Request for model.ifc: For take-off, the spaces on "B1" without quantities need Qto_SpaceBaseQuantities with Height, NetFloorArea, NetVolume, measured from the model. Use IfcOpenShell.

First a look at what the model holds.

```python
import ifcopenshell
import ifcopenshell.util.element
import ifcopenshell.util.unit

model = ifcopenshell.open("model.ifc")
print(model.schema)
for unit_type in ("LENGTHUNIT", "AREAUNIT", "VOLUMEUNIT"):
    print(unit_type, ifcopenshell.util.unit.calculate_unit_scale(model, unit_type))
storey = next(s for s in model.by_type("IfcBuildingStorey") if s.Name == "B1")
spaces = [e for e in ifcopenshell.util.element.get_decomposition(storey) if e.is_a("IfcSpace")]
for e in sorted(spaces, key=lambda e: e.id()):
    print(e.id(), e.is_a(), e.Name, list(ifcopenshell.util.element.get_psets(e, qtos_only=True)), sep=" | ")
```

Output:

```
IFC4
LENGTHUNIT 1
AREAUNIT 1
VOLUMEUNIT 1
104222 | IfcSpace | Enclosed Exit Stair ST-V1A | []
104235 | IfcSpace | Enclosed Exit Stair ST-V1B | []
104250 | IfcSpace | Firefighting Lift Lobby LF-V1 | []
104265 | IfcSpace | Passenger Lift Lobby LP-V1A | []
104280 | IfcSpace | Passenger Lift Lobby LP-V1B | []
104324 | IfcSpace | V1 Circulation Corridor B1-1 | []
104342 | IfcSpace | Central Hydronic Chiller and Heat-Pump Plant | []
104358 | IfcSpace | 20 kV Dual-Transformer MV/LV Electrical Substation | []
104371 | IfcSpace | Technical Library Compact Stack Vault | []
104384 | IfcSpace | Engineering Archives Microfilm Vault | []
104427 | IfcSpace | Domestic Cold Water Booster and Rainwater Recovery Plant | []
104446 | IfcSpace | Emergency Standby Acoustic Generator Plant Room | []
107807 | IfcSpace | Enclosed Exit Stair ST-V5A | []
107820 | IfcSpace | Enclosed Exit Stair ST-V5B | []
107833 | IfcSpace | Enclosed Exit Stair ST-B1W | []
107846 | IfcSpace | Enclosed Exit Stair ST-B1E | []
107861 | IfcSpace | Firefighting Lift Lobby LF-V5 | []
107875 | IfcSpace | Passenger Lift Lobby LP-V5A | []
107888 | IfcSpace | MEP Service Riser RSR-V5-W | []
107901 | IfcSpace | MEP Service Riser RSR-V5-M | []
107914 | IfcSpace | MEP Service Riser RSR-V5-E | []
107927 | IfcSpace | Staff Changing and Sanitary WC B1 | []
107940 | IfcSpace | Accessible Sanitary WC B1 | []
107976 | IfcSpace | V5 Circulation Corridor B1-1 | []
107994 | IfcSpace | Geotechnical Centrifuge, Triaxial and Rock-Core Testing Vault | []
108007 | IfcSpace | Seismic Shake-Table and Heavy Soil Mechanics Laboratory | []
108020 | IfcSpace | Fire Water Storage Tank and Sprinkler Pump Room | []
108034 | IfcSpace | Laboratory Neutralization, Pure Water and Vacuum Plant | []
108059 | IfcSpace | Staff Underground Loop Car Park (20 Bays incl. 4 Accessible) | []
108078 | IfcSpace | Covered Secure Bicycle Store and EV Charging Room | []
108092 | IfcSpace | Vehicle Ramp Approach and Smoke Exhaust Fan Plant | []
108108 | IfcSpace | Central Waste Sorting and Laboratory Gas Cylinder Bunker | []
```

```python
import ifcopenshell
import ifcopenshell.api.pset
import ifcopenshell.geom
import ifcopenshell.util.element
import ifcopenshell.util.shape
import ifcopenshell.util.unit

model = ifcopenshell.open("model.ifc")
unit_scale = ifcopenshell.util.unit.calculate_unit_scale(model)
area_scale = ifcopenshell.util.unit.calculate_unit_scale(model, "AREAUNIT")
volume_scale = ifcopenshell.util.unit.calculate_unit_scale(model, "VOLUMEUNIT")
settings = ifcopenshell.geom.settings()

storey = next(s for s in model.by_type("IfcBuildingStorey") if s.Name == "B1")
spaces = [e for e in ifcopenshell.util.element.get_decomposition(storey) if e.is_a("IfcSpace")]

for e in sorted(spaces, key=lambda e: e.id()):
    if ifcopenshell.util.element.get_psets(e, qtos_only=True, should_inherit=False):
        continue
    # Geometry comes back in metres, in the element's own axes.
    shape = ifcopenshell.geom.create_shape(settings, e)
    values = {
        "Height": ifcopenshell.util.shape.get_z(shape.geometry) / unit_scale,
        "NetFloorArea": ifcopenshell.util.shape.get_footprint_area(shape.geometry) / area_scale,
        "NetVolume": ifcopenshell.util.shape.get_volume(shape.geometry) / volume_scale,
    }
    qto = ifcopenshell.api.pset.add_qto(model, product=e, name="Qto_SpaceBaseQuantities")
    ifcopenshell.api.pset.edit_qto(model, qto=qto, properties=values)
    print(e.id(), {k: round(v, 3) for k, v in values.items()})

model.write("model_edited.ifc")
```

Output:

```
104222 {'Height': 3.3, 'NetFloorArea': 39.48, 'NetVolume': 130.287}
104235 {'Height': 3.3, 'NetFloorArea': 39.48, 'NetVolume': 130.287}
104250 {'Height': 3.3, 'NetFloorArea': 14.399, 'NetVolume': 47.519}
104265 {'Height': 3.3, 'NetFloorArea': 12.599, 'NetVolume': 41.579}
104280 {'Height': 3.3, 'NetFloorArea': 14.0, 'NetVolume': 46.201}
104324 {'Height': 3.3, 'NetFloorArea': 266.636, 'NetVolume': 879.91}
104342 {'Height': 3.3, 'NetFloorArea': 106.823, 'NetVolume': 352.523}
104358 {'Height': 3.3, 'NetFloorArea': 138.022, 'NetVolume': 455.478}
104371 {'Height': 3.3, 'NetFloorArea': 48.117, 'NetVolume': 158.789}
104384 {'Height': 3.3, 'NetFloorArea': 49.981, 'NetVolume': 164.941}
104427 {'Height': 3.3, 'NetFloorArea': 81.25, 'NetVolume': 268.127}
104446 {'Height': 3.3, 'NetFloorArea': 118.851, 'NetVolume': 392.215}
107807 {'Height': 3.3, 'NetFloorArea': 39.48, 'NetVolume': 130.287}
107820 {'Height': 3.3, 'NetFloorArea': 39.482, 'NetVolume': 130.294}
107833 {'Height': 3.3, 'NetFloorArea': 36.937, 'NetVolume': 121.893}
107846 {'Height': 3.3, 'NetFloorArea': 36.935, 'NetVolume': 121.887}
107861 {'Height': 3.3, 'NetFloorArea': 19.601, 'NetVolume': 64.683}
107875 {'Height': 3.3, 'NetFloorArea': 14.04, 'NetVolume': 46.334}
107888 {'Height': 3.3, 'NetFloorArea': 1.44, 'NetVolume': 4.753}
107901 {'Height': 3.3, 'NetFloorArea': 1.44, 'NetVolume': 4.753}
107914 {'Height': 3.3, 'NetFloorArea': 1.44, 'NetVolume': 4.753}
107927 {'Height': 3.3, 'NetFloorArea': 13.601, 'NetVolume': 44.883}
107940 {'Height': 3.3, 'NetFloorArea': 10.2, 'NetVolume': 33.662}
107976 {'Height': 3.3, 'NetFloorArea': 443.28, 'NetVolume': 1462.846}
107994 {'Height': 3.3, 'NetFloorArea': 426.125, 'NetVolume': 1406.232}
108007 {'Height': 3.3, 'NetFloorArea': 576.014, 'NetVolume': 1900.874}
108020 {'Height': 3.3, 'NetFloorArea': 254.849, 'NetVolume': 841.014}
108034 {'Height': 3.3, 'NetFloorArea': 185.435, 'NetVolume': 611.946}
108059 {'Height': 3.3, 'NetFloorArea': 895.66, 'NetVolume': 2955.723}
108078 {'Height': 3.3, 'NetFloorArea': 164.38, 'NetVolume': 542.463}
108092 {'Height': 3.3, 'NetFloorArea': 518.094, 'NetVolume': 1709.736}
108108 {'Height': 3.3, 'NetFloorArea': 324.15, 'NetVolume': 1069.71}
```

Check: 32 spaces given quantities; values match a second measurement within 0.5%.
